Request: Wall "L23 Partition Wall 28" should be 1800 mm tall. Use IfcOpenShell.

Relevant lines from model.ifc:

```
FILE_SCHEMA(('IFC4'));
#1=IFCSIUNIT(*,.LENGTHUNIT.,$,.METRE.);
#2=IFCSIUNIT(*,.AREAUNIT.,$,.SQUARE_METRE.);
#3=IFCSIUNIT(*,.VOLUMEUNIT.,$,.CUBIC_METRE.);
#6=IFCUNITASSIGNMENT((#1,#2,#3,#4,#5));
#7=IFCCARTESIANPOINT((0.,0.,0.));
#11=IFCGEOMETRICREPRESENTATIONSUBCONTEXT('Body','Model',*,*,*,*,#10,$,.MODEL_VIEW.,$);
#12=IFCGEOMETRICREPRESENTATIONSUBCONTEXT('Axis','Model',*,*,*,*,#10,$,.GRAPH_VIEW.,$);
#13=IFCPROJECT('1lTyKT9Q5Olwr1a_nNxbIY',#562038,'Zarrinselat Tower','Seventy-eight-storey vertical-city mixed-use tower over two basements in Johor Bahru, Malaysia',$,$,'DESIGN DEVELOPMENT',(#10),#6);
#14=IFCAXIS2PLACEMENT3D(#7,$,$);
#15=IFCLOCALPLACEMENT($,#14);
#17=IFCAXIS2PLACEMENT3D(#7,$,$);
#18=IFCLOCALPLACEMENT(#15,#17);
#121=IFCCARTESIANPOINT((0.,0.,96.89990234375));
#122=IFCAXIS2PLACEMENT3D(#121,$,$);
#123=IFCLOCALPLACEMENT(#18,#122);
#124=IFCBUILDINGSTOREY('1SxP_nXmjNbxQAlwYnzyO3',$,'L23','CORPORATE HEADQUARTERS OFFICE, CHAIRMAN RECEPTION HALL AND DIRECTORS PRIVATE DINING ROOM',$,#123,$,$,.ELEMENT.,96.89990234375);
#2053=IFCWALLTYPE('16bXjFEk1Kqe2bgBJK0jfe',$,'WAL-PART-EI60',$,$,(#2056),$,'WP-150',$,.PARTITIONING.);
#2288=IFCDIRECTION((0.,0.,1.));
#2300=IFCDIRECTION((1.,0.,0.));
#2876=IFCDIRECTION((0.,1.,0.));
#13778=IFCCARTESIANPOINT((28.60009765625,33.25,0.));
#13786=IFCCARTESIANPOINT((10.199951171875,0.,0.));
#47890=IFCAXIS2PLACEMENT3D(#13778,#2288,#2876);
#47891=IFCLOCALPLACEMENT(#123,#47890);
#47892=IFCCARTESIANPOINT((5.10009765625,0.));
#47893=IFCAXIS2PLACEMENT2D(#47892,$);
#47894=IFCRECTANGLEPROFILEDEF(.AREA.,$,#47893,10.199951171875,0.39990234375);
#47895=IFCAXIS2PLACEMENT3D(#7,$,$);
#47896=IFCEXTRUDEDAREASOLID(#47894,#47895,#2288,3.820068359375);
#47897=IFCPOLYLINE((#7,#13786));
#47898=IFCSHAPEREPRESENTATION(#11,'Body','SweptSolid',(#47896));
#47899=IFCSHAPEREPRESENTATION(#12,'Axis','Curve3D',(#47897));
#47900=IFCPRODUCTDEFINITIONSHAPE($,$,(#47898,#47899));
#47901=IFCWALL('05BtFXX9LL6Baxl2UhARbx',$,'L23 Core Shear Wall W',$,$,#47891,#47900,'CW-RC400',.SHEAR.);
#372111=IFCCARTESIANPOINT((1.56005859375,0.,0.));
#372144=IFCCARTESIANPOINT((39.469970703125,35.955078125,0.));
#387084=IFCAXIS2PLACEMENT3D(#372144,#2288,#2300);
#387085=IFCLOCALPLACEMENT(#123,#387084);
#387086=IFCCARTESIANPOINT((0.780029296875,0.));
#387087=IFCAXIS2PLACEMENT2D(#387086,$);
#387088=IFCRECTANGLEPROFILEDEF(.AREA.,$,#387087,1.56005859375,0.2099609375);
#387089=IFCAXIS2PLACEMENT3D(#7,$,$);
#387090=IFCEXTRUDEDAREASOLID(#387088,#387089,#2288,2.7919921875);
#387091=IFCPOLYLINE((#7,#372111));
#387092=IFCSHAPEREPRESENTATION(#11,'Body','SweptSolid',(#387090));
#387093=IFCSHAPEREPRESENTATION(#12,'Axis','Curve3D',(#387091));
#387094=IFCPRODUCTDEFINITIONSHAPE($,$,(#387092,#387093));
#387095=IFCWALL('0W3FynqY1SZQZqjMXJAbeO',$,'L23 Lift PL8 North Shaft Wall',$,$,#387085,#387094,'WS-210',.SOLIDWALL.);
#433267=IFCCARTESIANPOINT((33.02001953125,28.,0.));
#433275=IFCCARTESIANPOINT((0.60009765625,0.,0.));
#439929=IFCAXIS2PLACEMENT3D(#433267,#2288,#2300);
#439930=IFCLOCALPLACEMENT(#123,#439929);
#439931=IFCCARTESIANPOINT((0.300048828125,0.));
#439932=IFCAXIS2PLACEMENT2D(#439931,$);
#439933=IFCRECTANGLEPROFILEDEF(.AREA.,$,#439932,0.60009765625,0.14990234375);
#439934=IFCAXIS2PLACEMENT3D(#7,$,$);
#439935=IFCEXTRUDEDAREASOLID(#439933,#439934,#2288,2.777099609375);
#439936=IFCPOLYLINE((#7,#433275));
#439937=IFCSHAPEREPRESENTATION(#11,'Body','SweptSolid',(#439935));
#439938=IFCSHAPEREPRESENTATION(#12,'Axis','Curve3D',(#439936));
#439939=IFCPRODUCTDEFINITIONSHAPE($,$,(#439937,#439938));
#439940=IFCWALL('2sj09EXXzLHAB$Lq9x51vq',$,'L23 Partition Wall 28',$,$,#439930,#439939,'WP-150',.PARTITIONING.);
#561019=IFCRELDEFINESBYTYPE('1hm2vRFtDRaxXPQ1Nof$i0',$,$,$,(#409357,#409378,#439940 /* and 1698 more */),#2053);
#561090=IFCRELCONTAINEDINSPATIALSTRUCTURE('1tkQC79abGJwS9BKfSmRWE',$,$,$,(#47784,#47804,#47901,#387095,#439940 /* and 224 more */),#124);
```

```python
import ifcopenshell
import ifcopenshell.geom
import ifcopenshell.util.representation
import ifcopenshell.util.shape
import ifcopenshell.util.unit

model = ifcopenshell.open("model.ifc")
unit_scale = ifcopenshell.util.unit.calculate_unit_scale(model)
settings = ifcopenshell.geom.settings()


def volume(element):
    """Net volume in cubic metres, openings subtracted."""
    shape = ifcopenshell.geom.create_shape(settings, element)
    return ifcopenshell.util.shape.get_volume(shape.geometry)


wall = model.by_guid("2sj09EXXzLHAB$Lq9x51vq")
before = volume(wall)

body = ifcopenshell.util.representation.get_representation(wall, "Model", "Body")
solid = body.Items[0]
old_height = solid.Depth
solid.Depth = 1.8 / unit_scale
after = volume(wall)

print(f"height {old_height:g} -> {solid.Depth:g}, volume {before:.3f} -> {after:.3f} m3")

model.write("model_updated.ifc")
```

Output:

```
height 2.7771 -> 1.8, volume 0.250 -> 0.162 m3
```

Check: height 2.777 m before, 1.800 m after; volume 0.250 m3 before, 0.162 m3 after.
